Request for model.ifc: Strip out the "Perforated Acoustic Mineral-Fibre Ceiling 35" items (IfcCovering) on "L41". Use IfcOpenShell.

First a look at what the model holds.

```python
import ifcopenshell
import ifcopenshell.util.element

model = ifcopenshell.open("model.ifc")
print(model.schema)
storey = next(s for s in model.by_type("IfcBuildingStorey") if s.Name == "L41")
coverings = [e for e in ifcopenshell.util.element.get_decomposition(storey) if e.is_a("IfcCovering")]
seen = {}
for e in coverings:
    element_type = ifcopenshell.util.element.get_type(e)
    name = element_type.Name if element_type not in (None, e) else None
    seen[name] = seen.get(name, 0) + 1
for name, count in sorted(seen.items(), key=str):
    print(count, "x", name)
```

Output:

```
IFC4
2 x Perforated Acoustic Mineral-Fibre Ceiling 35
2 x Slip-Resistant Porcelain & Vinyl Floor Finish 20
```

```python
import ifcopenshell
import ifcopenshell.api.root
import ifcopenshell.util.element

model = ifcopenshell.open("model.ifc")

storey = next(s for s in model.by_type("IfcBuildingStorey") if s.Name == "L41")
coverings = [e for e in ifcopenshell.util.element.get_decomposition(storey) if e.is_a("IfcCovering")]
targets = [e for e in coverings if (t := ifcopenshell.util.element.get_type(e)) not in (None, e) and t.Name == "Perforated Acoustic Mineral-Fibre Ceiling 35"]

for e in targets:
    ifcopenshell.api.root.remove_product(model, product=e)
print(len(targets), "removed")

model.write("model_updated.ifc")
```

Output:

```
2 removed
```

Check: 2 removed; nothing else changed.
